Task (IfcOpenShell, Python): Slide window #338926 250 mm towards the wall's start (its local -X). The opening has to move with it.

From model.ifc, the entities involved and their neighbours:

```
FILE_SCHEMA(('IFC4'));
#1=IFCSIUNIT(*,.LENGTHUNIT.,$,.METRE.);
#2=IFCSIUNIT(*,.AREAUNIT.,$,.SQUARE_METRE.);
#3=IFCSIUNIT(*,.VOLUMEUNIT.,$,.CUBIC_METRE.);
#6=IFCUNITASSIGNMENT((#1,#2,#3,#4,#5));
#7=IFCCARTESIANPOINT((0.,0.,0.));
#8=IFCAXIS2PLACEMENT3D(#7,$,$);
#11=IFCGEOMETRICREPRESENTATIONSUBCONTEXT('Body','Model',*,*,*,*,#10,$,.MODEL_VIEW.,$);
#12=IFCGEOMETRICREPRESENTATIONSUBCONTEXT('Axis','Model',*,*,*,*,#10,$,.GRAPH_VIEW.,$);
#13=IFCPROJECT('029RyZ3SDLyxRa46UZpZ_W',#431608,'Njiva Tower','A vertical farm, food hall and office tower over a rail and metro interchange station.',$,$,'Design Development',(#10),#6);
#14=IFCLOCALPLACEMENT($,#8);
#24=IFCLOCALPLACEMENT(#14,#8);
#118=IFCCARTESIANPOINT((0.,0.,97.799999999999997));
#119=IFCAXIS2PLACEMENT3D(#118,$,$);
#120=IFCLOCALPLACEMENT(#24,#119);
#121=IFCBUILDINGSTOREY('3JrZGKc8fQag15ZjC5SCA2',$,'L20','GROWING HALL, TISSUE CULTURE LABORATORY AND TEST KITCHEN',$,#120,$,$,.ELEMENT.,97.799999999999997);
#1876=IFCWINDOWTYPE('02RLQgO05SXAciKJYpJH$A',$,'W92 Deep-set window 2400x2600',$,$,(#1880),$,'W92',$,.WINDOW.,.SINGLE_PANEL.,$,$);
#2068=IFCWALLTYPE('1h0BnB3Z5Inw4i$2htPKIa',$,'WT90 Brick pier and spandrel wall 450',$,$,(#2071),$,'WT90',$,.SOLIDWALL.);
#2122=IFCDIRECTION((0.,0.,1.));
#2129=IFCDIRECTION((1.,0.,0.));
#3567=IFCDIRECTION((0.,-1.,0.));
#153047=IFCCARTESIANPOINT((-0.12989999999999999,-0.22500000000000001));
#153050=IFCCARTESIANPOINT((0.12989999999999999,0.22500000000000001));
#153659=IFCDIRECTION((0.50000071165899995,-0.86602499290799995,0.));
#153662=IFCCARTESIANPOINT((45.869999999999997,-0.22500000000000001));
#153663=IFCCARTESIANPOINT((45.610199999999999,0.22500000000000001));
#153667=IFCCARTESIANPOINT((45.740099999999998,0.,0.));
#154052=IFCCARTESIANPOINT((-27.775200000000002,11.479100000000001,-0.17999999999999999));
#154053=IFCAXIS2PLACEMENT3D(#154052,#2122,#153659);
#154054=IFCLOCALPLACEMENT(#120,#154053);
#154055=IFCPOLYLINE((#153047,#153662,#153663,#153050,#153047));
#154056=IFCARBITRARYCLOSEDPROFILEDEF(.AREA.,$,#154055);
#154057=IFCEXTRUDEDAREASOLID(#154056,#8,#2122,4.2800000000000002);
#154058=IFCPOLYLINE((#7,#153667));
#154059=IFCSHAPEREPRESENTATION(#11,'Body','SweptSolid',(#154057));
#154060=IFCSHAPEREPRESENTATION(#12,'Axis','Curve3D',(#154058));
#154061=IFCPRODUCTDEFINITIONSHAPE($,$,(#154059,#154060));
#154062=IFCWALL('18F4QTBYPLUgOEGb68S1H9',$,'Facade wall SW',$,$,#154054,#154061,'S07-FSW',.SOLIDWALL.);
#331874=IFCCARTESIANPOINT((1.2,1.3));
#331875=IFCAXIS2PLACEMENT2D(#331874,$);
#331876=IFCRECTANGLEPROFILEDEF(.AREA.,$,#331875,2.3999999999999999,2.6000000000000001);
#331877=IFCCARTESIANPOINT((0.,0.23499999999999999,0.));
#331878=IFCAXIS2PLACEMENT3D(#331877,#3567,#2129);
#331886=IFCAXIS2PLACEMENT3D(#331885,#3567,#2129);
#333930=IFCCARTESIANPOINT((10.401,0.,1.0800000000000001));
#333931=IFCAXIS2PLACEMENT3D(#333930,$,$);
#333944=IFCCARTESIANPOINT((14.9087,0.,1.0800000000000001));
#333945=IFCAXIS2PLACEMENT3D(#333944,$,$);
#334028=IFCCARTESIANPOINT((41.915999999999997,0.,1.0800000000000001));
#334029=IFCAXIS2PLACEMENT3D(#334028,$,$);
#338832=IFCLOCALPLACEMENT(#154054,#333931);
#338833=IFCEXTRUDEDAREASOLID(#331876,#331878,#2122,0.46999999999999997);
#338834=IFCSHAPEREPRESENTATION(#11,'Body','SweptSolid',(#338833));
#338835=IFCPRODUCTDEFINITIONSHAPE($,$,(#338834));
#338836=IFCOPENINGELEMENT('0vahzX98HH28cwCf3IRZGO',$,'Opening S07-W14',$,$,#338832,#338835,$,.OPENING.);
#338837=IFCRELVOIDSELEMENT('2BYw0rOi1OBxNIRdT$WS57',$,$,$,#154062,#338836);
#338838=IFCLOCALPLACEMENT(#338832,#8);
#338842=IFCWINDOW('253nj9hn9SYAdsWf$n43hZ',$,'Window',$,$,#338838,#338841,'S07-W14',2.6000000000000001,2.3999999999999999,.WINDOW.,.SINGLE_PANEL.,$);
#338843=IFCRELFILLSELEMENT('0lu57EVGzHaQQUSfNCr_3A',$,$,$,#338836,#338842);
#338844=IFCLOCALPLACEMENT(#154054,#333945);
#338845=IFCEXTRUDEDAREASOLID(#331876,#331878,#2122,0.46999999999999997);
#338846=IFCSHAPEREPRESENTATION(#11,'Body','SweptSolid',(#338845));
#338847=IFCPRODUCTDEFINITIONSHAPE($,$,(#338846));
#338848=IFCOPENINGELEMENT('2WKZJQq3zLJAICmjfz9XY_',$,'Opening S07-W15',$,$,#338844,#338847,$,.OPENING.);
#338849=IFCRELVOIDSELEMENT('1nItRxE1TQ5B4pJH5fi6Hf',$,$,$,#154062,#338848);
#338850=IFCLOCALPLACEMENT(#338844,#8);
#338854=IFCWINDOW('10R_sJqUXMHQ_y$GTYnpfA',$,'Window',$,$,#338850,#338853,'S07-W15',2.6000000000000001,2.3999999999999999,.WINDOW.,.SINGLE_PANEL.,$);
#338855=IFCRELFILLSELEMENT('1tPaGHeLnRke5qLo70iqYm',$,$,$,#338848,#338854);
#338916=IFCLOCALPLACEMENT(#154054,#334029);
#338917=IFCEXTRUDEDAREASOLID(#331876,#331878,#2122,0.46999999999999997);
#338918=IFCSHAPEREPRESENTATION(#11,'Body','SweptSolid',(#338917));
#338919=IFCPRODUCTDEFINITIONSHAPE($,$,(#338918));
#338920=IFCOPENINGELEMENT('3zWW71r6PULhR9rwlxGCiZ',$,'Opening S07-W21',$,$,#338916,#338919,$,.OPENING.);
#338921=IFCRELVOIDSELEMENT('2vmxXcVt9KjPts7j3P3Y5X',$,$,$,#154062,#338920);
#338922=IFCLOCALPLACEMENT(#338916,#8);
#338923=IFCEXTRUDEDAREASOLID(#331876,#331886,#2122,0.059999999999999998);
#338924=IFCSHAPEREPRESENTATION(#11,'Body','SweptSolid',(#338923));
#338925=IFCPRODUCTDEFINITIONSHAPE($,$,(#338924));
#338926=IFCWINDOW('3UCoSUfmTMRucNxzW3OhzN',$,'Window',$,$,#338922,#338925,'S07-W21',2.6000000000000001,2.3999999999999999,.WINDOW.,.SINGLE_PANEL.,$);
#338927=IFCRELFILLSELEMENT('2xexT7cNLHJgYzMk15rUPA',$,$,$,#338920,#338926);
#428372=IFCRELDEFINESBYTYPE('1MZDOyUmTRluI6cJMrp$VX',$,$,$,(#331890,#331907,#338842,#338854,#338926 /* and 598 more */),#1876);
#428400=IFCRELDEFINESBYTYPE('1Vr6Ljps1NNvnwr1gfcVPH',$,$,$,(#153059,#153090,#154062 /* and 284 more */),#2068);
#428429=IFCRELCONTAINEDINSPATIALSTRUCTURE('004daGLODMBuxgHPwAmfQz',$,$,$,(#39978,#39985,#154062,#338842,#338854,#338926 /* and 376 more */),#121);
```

```python
import ifcopenshell
import ifcopenshell.api.geometry
import ifcopenshell.util.placement
import ifcopenshell.util.unit

model = ifcopenshell.open("model.ifc")
unit_scale = ifcopenshell.util.unit.calculate_unit_scale(model)

window = model.by_guid("3UCoSUfmTMRucNxzW3OhzN")
opening = window.FillsVoids[0].RelatingOpeningElement
wall = opening.VoidsElements[0].RelatingBuildingElement

wall_matrix = ifcopenshell.util.placement.get_local_placement(wall.ObjectPlacement)
shift = wall_matrix[:3, 0] * -0.25 / unit_scale
before = ifcopenshell.util.placement.get_local_placement(window.ObjectPlacement)[:3, 3].copy()

# The window is placed relative to its opening, so it follows when the opening moves.
matrix = ifcopenshell.util.placement.get_local_placement(opening.ObjectPlacement)
matrix[:3, 3] += shift
ifcopenshell.api.geometry.edit_object_placement(
    model, product=opening, matrix=matrix, is_si=False, should_transform_children=True
)

after = ifcopenshell.util.placement.get_local_placement(window.ObjectPlacement)[:3, 3]
print("window moved by", (after - before).round(3) + 0.0)

model.write("model_edited.ifc")
```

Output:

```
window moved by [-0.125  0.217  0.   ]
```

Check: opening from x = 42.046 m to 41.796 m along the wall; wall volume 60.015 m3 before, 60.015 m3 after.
